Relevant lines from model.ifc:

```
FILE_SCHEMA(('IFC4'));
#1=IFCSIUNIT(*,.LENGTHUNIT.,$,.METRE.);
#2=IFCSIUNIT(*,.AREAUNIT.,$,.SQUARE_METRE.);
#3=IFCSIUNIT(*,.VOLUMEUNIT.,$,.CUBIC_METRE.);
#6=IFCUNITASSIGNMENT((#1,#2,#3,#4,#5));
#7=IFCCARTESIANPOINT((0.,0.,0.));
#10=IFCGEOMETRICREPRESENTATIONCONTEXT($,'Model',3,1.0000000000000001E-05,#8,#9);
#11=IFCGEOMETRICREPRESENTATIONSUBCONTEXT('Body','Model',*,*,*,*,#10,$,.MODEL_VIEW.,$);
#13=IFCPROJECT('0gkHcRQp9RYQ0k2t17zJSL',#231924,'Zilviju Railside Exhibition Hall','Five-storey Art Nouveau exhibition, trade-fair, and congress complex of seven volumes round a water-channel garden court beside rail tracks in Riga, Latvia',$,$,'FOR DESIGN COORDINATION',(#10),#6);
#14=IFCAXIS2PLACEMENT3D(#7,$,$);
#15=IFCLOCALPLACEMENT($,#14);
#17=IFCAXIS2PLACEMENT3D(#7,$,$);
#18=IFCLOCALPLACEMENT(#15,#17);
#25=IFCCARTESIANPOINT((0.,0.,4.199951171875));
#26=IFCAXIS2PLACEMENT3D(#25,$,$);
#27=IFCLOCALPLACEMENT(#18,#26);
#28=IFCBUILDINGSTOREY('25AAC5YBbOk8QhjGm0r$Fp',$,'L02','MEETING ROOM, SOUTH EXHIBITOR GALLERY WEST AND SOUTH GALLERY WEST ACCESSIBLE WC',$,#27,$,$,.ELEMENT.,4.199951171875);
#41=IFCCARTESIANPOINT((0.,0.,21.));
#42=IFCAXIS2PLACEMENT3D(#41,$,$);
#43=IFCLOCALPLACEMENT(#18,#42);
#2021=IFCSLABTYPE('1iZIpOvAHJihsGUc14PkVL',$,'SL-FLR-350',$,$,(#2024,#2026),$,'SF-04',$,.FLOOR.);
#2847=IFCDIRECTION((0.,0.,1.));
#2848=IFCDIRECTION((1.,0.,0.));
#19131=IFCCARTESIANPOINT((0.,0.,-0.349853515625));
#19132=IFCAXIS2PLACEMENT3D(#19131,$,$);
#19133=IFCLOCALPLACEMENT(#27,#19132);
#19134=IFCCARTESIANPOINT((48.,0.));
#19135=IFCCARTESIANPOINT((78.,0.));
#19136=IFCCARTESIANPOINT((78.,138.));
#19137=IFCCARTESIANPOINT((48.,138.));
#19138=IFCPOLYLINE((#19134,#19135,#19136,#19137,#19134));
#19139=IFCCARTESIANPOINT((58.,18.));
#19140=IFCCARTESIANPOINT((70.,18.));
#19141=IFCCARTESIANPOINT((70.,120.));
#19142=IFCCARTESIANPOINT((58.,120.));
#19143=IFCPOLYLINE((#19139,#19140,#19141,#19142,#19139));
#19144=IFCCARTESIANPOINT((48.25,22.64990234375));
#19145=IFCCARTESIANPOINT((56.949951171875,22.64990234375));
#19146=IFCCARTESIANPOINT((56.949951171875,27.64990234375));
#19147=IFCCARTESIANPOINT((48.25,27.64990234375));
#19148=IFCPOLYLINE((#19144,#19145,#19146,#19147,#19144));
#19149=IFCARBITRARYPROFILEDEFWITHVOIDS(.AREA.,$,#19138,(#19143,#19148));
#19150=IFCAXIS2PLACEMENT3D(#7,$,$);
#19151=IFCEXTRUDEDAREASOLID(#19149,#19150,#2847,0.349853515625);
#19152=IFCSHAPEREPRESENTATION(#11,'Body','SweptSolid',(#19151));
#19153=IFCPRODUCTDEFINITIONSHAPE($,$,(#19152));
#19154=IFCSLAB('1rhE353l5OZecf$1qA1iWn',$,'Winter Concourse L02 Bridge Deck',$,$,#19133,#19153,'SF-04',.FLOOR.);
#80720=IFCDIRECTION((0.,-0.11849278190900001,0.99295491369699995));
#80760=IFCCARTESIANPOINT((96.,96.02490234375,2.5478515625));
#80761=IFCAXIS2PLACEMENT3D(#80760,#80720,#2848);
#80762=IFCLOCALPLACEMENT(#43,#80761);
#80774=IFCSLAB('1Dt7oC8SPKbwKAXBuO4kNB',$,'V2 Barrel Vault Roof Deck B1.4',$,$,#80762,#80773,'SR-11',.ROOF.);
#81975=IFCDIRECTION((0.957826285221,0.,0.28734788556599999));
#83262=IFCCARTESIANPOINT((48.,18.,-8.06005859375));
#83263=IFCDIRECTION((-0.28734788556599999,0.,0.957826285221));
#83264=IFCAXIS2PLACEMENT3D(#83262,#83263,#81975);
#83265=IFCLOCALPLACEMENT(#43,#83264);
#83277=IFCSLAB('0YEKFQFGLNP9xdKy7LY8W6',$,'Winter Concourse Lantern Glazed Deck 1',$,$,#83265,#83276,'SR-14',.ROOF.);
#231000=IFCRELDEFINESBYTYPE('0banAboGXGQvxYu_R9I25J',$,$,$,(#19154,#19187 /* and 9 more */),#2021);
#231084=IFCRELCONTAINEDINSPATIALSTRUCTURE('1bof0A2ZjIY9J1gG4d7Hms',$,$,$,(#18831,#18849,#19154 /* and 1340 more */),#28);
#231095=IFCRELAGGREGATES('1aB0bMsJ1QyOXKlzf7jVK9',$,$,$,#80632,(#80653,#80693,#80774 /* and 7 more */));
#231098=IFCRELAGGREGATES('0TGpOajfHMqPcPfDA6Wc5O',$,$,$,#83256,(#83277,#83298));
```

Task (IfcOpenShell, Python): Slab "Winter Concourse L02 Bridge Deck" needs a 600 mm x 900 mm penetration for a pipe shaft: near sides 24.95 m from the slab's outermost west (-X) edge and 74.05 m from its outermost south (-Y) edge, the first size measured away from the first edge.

```python
import numpy as np
import ifcopenshell
import ifcopenshell.api.feature
import ifcopenshell.api.geometry
import ifcopenshell.api.root
import ifcopenshell.geom
import ifcopenshell.util.placement
import ifcopenshell.util.representation
import ifcopenshell.util.shape
import ifcopenshell.util.unit

model = ifcopenshell.open("model.ifc")
unit_scale = ifcopenshell.util.unit.calculate_unit_scale(model)
settings = ifcopenshell.geom.settings()


def volume(element):
    """Net volume in cubic metres, openings subtracted."""
    shape = ifcopenshell.geom.create_shape(settings, element)
    return ifcopenshell.util.shape.get_volume(shape.geometry)


slab = model.by_guid("1rhE353l5OZecf$1qA1iWn")
before = volume(slab)

# Extent in the slab's own axes, in metres. The edges named are its -X and -Y sides.
slab_shape = ifcopenshell.geom.create_shape(settings, slab)
vertices = ifcopenshell.util.shape.get_vertices(slab_shape.geometry)
x_min, y_min, bottom = vertices.min(axis=0)
top = vertices[:, 2].max()

opening = ifcopenshell.api.root.create_entity(model, ifc_class="IfcOpeningElement", name="Pipe shaft opening", predefined_type="OPENING")
context = ifcopenshell.util.representation.get_context(model, "Model", "Body", "MODEL_VIEW")
width, depth = 0.6, 0.9
outline = [(0.0, 0.0), (width, 0.0), (width, depth), (0.0, depth), (0.0, 0.0)]
# Overshoot both faces by 50 mm so the cut is clean.
shape = ifcopenshell.api.geometry.add_slab_representation(
    model, context=context, depth=top - bottom + 0.1, polyline=outline
)
ifcopenshell.api.geometry.assign_representation(model, product=opening, representation=shape)

matrix = ifcopenshell.util.placement.get_local_placement(slab.ObjectPlacement)
matrix[:, 3] = matrix @ np.append(np.array([x_min + 24.95, y_min + 74.05, bottom - 0.05]) / unit_scale, 1.0)
ifcopenshell.api.geometry.edit_object_placement(model, product=opening, matrix=matrix, is_si=False)
ifcopenshell.api.feature.add_feature(model, feature=opening, element=slab)

after = volume(slab)

print(f"slab volume {before:.3f} -> {after:.3f} m3")

model.write("model_edited.ifc")
```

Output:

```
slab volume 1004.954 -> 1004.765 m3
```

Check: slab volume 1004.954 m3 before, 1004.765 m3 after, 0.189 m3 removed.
